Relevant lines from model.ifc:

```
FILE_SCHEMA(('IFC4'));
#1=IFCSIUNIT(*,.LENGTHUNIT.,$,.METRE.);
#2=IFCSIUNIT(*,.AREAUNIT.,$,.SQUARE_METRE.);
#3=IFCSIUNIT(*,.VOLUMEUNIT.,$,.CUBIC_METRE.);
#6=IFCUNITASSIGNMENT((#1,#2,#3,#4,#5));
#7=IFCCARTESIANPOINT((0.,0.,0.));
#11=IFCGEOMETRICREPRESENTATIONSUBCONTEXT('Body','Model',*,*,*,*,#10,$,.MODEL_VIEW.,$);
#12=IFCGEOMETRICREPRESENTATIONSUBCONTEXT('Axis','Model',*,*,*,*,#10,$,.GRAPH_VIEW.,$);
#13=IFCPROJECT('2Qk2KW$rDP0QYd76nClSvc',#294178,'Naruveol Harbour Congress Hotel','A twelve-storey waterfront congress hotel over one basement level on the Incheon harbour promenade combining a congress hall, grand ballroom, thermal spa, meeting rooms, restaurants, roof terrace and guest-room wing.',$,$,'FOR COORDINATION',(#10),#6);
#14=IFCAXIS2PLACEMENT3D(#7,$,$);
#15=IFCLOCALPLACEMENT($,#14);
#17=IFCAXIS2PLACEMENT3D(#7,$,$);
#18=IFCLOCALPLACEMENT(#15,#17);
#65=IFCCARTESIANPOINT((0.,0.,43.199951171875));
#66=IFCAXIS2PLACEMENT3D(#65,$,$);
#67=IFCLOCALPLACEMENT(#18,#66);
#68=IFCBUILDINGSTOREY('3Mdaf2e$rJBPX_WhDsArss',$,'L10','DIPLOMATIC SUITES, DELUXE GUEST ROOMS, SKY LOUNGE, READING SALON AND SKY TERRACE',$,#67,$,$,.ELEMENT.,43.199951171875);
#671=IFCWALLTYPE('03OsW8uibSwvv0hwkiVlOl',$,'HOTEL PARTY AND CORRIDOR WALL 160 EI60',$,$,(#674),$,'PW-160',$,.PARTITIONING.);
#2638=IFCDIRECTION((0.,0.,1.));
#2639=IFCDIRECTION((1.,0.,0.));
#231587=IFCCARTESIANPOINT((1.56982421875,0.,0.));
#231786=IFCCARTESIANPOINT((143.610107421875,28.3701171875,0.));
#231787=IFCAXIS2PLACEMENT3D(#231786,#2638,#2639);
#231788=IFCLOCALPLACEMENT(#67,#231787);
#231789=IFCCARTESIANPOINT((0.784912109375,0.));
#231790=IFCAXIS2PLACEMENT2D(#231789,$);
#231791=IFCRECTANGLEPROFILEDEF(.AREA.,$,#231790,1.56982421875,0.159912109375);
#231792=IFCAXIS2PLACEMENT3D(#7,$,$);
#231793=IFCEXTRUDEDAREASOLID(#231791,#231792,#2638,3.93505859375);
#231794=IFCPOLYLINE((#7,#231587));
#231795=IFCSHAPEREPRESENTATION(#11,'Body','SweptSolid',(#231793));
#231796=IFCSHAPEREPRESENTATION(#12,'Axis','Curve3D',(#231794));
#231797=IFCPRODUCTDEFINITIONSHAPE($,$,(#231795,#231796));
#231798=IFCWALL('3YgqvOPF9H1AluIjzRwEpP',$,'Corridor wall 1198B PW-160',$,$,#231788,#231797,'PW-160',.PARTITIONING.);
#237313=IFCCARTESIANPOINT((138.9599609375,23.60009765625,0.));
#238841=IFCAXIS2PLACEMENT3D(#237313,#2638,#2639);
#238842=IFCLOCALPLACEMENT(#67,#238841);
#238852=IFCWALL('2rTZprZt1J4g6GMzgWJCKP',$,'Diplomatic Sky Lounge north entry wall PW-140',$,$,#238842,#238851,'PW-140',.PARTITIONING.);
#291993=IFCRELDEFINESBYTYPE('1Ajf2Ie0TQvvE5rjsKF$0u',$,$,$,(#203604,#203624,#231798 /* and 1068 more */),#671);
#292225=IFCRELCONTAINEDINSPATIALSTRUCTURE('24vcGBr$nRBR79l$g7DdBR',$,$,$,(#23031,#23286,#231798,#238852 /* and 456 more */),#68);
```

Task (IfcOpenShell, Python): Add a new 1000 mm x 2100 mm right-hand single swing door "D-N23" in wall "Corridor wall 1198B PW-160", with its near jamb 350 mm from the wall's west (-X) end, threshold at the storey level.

```python
import numpy as np
import ifcopenshell
import ifcopenshell.api.feature
import ifcopenshell.api.geometry
import ifcopenshell.api.root
import ifcopenshell.api.spatial
import ifcopenshell.geom
import ifcopenshell.util.element
import ifcopenshell.util.placement
import ifcopenshell.util.representation
import ifcopenshell.util.shape
import ifcopenshell.util.unit

model = ifcopenshell.open("model.ifc")
unit_scale = ifcopenshell.util.unit.calculate_unit_scale(model)
settings = ifcopenshell.geom.settings()


def volume(element):
    """Net volume in cubic metres, openings subtracted."""
    shape = ifcopenshell.geom.create_shape(settings, element)
    return ifcopenshell.util.shape.get_volume(shape.geometry)


wall = model.by_guid("3YgqvOPF9H1AluIjzRwEpP")
storey = ifcopenshell.util.element.get_container(wall, ifc_class="IfcBuildingStorey")
context = ifcopenshell.util.representation.get_context(model, "Model", "Body", "MODEL_VIEW")
before = volume(wall)

width, height, from_end, sill = 1, 2.1, 0.35, 0.0  # metres

# The wall runs along its own X axis, and the end named is its -X end.
wall_shape = ifcopenshell.geom.create_shape(settings, wall)
x, y, z = ifcopenshell.util.shape.get_vertices(wall_shape.geometry).T
start = x.min() + from_end
face, thickness = float(y.min()), float(y.max() - y.min())
wall_matrix = ifcopenshell.util.placement.get_local_placement(wall.ObjectPlacement)
level = ifcopenshell.util.placement.get_local_placement(storey.ObjectPlacement)[2, 3]


def in_wall(x, y):
    """Placement at x, y metres in the wall's axes, at sill height."""
    matrix = wall_matrix.copy()
    matrix[:, 3] = wall_matrix @ np.array([x / unit_scale, y / unit_scale, 0.0, 1.0])
    matrix[2, 3] = level + sill / unit_scale
    return matrix


# Opening: a box that overshoots both wall faces by 50 mm.
opening = ifcopenshell.api.root.create_entity(model, ifc_class="IfcOpeningElement", predefined_type="OPENING")
box = ifcopenshell.api.geometry.add_wall_representation(
    model, context=context, length=width, height=height, thickness=thickness + 0.1
)
ifcopenshell.api.geometry.assign_representation(model, product=opening, representation=box)
ifcopenshell.api.geometry.edit_object_placement(model, product=opening, matrix=in_wall(start, face - 0.05), is_si=False)
ifcopenshell.api.feature.add_feature(model, feature=opening, element=wall)

door = ifcopenshell.api.root.create_entity(model, ifc_class="IfcDoor", name="D-N23", predefined_type="DOOR")
door.OverallWidth, door.OverallHeight = width / unit_scale, height / unit_scale
door.OperationType = "SINGLE_SWING_RIGHT"
body = ifcopenshell.api.geometry.add_door_representation(
    model,
    context=context,
    overall_width=door.OverallWidth,
    overall_height=door.OverallHeight,
    operation_type="SINGLE_SWING_RIGHT",
    lining_properties={"LiningDepth": thickness / unit_scale, "ThresholdDepth": thickness / unit_scale},
)
ifcopenshell.api.geometry.assign_representation(model, product=door, representation=body)
ifcopenshell.api.spatial.assign_container(model, products=[door], relating_structure=storey)
ifcopenshell.api.feature.add_filling(model, opening=opening, element=door)

# The lining spans the wall, so the door starts at the wall face.
ifcopenshell.api.geometry.edit_object_placement(model, product=door, matrix=in_wall(start, face), is_si=False)

after = volume(wall)

print(f"wall volume {before:.3f} -> {after:.3f} m3")

model.write("model-out.ifc")
```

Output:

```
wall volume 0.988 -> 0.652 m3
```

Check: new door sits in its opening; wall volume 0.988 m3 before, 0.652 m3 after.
